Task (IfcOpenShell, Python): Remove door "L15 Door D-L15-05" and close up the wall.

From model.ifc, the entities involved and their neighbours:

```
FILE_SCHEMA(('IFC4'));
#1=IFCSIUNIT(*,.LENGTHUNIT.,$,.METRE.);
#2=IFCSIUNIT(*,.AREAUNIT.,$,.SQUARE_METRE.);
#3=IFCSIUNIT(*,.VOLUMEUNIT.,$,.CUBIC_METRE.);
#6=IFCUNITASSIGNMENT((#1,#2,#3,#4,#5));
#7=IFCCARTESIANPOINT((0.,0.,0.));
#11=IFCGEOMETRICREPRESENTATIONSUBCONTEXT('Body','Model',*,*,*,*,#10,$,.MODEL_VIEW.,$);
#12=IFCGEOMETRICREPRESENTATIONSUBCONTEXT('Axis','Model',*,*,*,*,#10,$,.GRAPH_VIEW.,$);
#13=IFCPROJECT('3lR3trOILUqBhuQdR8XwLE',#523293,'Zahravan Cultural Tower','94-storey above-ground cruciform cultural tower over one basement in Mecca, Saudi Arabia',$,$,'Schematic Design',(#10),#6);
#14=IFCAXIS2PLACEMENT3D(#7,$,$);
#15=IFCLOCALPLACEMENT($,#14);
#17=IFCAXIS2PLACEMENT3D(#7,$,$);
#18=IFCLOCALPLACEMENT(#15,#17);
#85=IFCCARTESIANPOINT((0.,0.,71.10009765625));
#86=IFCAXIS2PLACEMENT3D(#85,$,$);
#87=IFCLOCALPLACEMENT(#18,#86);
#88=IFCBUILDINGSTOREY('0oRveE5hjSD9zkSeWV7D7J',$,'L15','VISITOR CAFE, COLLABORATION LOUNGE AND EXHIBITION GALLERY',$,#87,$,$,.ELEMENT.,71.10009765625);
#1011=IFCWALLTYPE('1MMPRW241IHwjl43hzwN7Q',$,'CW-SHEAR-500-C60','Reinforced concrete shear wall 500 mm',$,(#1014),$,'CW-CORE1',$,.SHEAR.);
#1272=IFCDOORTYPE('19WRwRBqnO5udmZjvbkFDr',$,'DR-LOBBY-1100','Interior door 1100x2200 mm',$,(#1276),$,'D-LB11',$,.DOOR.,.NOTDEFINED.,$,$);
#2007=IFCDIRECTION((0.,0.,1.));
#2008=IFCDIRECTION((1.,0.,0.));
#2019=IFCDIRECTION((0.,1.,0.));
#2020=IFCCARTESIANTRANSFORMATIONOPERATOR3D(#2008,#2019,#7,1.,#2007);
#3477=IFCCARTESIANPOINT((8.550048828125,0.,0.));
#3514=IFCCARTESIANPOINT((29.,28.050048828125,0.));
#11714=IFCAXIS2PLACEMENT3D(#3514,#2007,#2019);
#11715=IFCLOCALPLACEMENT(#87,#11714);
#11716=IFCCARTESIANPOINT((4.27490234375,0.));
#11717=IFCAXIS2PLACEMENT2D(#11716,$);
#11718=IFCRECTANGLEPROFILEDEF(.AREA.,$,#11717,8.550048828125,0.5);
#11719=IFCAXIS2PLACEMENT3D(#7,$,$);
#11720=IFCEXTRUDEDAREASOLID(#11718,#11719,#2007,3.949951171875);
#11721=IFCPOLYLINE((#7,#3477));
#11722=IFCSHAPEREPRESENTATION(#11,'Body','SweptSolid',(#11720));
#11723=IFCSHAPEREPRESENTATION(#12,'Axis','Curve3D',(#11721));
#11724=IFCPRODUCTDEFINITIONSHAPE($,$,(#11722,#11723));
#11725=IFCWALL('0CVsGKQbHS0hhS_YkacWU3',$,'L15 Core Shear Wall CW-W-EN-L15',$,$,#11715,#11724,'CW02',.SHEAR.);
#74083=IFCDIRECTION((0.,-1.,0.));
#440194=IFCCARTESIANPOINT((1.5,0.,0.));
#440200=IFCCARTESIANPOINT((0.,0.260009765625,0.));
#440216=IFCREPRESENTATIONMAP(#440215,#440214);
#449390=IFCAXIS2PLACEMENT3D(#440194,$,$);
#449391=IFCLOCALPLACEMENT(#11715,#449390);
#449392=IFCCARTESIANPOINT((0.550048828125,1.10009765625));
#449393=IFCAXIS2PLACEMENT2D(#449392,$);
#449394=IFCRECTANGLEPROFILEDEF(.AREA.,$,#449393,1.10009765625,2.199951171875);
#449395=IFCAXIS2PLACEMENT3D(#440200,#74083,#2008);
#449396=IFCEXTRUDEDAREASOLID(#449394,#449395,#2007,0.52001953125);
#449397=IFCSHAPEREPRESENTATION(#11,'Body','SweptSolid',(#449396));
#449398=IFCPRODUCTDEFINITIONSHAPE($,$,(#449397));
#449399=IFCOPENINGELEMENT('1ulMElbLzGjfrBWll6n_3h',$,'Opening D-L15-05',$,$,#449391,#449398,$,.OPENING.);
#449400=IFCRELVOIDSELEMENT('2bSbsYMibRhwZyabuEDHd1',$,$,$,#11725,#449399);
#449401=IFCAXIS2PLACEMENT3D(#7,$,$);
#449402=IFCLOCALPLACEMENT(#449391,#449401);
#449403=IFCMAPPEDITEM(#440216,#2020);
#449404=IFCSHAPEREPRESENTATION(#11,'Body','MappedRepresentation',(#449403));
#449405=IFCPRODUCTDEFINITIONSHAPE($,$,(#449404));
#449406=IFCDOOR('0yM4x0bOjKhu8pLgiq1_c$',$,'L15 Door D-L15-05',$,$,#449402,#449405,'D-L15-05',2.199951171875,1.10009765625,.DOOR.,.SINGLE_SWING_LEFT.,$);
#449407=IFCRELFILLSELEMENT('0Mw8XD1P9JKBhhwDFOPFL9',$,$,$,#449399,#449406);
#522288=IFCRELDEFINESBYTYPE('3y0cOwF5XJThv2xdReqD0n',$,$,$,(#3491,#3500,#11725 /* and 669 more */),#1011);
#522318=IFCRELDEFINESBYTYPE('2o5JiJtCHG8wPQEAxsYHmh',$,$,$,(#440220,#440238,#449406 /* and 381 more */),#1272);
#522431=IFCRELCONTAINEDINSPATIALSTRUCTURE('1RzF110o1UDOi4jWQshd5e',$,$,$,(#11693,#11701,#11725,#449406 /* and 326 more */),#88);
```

```python
import ifcopenshell
import ifcopenshell.api.feature
import ifcopenshell.api.root
import ifcopenshell.geom
import ifcopenshell.util.shape

model = ifcopenshell.open("model.ifc")
settings = ifcopenshell.geom.settings()


def volume(element):
    """Net volume in cubic metres, openings subtracted."""
    shape = ifcopenshell.geom.create_shape(settings, element)
    return ifcopenshell.util.shape.get_volume(shape.geometry)


door = model.by_guid("0yM4x0bOjKhu8pLgiq1_c$")
opening = door.FillsVoids[0].RelatingOpeningElement
wall = opening.VoidsElements[0].RelatingBuildingElement
before = volume(wall)

ifcopenshell.api.root.remove_product(model, product=door)
ifcopenshell.api.feature.remove_feature(model, feature=opening)

after = volume(wall)

print(f"wall volume {before:.3f} -> {after:.3f} m3")

model.write("model-out.ifc")
```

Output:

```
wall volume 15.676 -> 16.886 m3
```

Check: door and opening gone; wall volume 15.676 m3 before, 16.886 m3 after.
